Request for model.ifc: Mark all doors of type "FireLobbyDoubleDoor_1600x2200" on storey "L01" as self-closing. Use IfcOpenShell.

First a look at what the model holds.

```python
import ifcopenshell
import ifcopenshell.util.element

model = ifcopenshell.open("model.ifc")
print(model.schema)
storey = next(s for s in model.by_type("IfcBuildingStorey") if s.Name == "L01")
doors = [e for e in ifcopenshell.util.element.get_decomposition(storey) if e.is_a("IfcDoor")]
seen = {}
for e in doors:
    element_type = ifcopenshell.util.element.get_type(e)
    key = (element_type.Name if element_type != e and element_type else None, ifcopenshell.util.element.get_pset(e, "Pset_DoorCommon", "SelfClosing"))
    seen[key] = seen.get(key, 0) + 1
for (name, value), count in sorted(seen.items(), key=str):
    print(count, "x", name, "|", value)
```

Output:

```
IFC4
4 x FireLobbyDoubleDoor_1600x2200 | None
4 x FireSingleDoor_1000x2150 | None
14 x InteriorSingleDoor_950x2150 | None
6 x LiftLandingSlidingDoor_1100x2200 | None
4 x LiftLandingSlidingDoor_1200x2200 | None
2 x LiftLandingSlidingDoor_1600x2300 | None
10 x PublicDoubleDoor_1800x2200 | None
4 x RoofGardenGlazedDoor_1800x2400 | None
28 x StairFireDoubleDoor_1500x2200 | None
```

```python
import ifcopenshell
import ifcopenshell.api.pset
import ifcopenshell.util.element

model = ifcopenshell.open("model.ifc")

storey = next(s for s in model.by_type("IfcBuildingStorey") if s.Name == "L01")
doors = [e for e in ifcopenshell.util.element.get_decomposition(storey) if e.is_a("IfcDoor")]

count = 0
for e in doors:
    element_type = ifcopenshell.util.element.get_type(e)
    if element_type in (None, e) or element_type.Name != "FireLobbyDoubleDoor_1600x2200":
        continue
    # add_pset returns the element's existing set when there is one.
    pset = ifcopenshell.api.pset.add_pset(model, product=e, name="Pset_DoorCommon")
    ifcopenshell.api.pset.edit_pset(model, pset=pset, properties={"SelfClosing": True})
    count += 1

print(count, "doors updated")

model.write("model_rev.ifc")
```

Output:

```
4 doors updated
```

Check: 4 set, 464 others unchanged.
